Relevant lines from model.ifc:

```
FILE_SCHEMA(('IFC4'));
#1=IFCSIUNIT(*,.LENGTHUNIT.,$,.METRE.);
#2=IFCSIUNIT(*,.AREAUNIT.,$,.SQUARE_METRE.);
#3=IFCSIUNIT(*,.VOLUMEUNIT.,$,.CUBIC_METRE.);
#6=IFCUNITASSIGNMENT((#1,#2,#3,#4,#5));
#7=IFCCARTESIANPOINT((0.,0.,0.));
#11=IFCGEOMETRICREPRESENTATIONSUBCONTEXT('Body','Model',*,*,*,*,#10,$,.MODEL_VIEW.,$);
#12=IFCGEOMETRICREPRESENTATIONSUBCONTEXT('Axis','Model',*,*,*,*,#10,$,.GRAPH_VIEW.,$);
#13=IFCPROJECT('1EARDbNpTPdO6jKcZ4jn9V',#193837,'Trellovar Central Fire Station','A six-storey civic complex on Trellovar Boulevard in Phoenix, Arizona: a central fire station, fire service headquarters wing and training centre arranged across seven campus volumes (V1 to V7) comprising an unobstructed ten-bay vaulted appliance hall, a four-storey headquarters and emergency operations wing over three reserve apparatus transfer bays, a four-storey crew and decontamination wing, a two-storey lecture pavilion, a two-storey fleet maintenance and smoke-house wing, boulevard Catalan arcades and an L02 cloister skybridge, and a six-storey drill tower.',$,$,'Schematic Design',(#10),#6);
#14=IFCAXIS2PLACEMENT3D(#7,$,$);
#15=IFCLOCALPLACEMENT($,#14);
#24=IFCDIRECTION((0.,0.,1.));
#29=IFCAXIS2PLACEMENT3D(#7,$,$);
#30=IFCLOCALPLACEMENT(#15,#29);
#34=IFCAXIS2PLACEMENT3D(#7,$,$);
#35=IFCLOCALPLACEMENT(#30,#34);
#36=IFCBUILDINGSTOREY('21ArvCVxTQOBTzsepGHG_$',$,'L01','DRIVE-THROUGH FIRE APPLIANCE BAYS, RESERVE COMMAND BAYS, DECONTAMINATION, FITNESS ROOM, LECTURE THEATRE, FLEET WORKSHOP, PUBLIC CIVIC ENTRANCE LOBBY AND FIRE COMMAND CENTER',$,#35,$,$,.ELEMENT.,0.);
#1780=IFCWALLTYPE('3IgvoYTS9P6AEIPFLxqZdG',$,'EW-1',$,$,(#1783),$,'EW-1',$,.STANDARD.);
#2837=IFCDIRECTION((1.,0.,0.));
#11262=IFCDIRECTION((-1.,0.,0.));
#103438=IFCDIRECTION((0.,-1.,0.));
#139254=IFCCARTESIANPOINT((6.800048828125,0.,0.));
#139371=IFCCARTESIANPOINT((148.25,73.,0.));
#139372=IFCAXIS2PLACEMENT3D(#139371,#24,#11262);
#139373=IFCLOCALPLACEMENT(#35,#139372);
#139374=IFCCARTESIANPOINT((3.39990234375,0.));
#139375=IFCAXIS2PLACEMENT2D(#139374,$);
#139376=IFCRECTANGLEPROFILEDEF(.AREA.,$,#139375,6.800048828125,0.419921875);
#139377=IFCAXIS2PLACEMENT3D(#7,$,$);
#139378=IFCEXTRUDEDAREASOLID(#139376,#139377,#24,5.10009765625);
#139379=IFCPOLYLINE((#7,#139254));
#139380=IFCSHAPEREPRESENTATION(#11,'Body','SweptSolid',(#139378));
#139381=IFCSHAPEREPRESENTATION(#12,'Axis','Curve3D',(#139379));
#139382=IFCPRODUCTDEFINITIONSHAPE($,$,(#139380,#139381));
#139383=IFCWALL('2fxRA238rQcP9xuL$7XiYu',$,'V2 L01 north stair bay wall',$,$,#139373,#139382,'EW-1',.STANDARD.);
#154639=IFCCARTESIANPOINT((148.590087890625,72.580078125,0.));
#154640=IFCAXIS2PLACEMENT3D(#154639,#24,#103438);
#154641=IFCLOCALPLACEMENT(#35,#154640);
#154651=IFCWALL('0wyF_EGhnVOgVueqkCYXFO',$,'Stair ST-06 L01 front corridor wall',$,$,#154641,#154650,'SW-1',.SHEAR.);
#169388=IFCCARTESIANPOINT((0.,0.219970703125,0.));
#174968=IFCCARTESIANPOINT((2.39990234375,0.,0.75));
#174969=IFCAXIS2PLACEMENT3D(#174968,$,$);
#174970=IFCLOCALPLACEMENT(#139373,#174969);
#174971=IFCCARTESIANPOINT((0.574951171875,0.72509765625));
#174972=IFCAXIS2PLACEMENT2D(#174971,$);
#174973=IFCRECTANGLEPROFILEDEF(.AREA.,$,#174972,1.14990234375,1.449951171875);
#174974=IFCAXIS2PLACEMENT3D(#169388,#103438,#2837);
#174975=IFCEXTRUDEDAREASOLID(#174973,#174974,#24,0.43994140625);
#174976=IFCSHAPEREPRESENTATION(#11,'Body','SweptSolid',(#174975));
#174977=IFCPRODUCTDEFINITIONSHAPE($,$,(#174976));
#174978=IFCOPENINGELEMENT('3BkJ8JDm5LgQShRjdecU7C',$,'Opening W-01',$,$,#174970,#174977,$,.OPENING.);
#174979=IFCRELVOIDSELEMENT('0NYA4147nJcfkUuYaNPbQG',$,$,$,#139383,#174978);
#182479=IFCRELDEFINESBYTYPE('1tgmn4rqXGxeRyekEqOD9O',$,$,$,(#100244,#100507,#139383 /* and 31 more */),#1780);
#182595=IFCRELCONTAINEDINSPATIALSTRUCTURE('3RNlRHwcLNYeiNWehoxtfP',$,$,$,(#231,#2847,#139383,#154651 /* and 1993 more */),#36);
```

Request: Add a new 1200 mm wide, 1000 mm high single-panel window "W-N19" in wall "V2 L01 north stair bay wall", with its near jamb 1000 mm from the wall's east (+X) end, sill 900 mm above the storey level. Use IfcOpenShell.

```python
import numpy as np
import ifcopenshell
import ifcopenshell.api.feature
import ifcopenshell.api.geometry
import ifcopenshell.api.root
import ifcopenshell.api.spatial
import ifcopenshell.geom
import ifcopenshell.util.element
import ifcopenshell.util.placement
import ifcopenshell.util.representation
import ifcopenshell.util.shape
import ifcopenshell.util.unit

model = ifcopenshell.open("model.ifc")
unit_scale = ifcopenshell.util.unit.calculate_unit_scale(model)
settings = ifcopenshell.geom.settings()


def volume(element):
    """Net volume in cubic metres, openings subtracted."""
    shape = ifcopenshell.geom.create_shape(settings, element)
    return ifcopenshell.util.shape.get_volume(shape.geometry)


wall = model.by_id(139383)
storey = ifcopenshell.util.element.get_container(wall, ifc_class="IfcBuildingStorey")
context = ifcopenshell.util.representation.get_context(model, "Model", "Body", "MODEL_VIEW")
before = volume(wall)

width, height, from_end, sill = 1.2, 1, 1, 0.9  # metres

# The wall runs along its own X axis, and the end named is its -X end.
wall_shape = ifcopenshell.geom.create_shape(settings, wall)
x, y, z = ifcopenshell.util.shape.get_vertices(wall_shape.geometry).T
start = x.min() + from_end
face, thickness = float(y.min()), float(y.max() - y.min())
wall_matrix = ifcopenshell.util.placement.get_local_placement(wall.ObjectPlacement)
level = ifcopenshell.util.placement.get_local_placement(storey.ObjectPlacement)[2, 3]


def in_wall(x, y):
    """Placement at x, y metres in the wall's axes, at sill height."""
    matrix = wall_matrix.copy()
    matrix[:, 3] = wall_matrix @ np.array([x / unit_scale, y / unit_scale, 0.0, 1.0])
    matrix[2, 3] = level + sill / unit_scale
    return matrix


# Opening: a box that overshoots both wall faces by 50 mm.
opening = ifcopenshell.api.root.create_entity(model, ifc_class="IfcOpeningElement", predefined_type="OPENING")
box = ifcopenshell.api.geometry.add_wall_representation(
    model, context=context, length=width, height=height, thickness=thickness + 0.1
)
ifcopenshell.api.geometry.assign_representation(model, product=opening, representation=box)
ifcopenshell.api.geometry.edit_object_placement(model, product=opening, matrix=in_wall(start, face - 0.05), is_si=False)
ifcopenshell.api.feature.add_feature(model, feature=opening, element=wall)

window = ifcopenshell.api.root.create_entity(model, ifc_class="IfcWindow", name="W-N19", predefined_type="WINDOW")
window.OverallWidth, window.OverallHeight = width / unit_scale, height / unit_scale
window.PartitioningType = "SINGLE_PANEL"
body = ifcopenshell.api.geometry.add_window_representation(
    model,
    context=context,
    overall_width=window.OverallWidth,
    overall_height=window.OverallHeight,
    partition_type="SINGLE_PANEL",
)
ifcopenshell.api.geometry.assign_representation(model, product=window, representation=body)
ifcopenshell.api.spatial.assign_container(model, products=[window], relating_structure=storey)
ifcopenshell.api.feature.add_filling(model, opening=opening, element=window)

# Centre the window in the wall's thickness.
ifcopenshell.api.geometry.edit_object_placement(model, product=window, matrix=in_wall(start, face), is_si=False)
window_shape = ifcopenshell.geom.create_shape(settings, window)
depth = ifcopenshell.util.shape.get_vertices(window_shape.geometry)[:, 1]
offset = face + thickness / 2 - (depth.min() + depth.max()) / 2
ifcopenshell.api.geometry.edit_object_placement(model, product=window, matrix=in_wall(start, offset), is_si=False)

after = volume(wall)

print(f"wall volume {before:.3f} -> {after:.3f} m3")

model.write("model-out.ifc")
```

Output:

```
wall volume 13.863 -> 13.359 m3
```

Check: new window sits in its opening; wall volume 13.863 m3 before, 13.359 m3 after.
